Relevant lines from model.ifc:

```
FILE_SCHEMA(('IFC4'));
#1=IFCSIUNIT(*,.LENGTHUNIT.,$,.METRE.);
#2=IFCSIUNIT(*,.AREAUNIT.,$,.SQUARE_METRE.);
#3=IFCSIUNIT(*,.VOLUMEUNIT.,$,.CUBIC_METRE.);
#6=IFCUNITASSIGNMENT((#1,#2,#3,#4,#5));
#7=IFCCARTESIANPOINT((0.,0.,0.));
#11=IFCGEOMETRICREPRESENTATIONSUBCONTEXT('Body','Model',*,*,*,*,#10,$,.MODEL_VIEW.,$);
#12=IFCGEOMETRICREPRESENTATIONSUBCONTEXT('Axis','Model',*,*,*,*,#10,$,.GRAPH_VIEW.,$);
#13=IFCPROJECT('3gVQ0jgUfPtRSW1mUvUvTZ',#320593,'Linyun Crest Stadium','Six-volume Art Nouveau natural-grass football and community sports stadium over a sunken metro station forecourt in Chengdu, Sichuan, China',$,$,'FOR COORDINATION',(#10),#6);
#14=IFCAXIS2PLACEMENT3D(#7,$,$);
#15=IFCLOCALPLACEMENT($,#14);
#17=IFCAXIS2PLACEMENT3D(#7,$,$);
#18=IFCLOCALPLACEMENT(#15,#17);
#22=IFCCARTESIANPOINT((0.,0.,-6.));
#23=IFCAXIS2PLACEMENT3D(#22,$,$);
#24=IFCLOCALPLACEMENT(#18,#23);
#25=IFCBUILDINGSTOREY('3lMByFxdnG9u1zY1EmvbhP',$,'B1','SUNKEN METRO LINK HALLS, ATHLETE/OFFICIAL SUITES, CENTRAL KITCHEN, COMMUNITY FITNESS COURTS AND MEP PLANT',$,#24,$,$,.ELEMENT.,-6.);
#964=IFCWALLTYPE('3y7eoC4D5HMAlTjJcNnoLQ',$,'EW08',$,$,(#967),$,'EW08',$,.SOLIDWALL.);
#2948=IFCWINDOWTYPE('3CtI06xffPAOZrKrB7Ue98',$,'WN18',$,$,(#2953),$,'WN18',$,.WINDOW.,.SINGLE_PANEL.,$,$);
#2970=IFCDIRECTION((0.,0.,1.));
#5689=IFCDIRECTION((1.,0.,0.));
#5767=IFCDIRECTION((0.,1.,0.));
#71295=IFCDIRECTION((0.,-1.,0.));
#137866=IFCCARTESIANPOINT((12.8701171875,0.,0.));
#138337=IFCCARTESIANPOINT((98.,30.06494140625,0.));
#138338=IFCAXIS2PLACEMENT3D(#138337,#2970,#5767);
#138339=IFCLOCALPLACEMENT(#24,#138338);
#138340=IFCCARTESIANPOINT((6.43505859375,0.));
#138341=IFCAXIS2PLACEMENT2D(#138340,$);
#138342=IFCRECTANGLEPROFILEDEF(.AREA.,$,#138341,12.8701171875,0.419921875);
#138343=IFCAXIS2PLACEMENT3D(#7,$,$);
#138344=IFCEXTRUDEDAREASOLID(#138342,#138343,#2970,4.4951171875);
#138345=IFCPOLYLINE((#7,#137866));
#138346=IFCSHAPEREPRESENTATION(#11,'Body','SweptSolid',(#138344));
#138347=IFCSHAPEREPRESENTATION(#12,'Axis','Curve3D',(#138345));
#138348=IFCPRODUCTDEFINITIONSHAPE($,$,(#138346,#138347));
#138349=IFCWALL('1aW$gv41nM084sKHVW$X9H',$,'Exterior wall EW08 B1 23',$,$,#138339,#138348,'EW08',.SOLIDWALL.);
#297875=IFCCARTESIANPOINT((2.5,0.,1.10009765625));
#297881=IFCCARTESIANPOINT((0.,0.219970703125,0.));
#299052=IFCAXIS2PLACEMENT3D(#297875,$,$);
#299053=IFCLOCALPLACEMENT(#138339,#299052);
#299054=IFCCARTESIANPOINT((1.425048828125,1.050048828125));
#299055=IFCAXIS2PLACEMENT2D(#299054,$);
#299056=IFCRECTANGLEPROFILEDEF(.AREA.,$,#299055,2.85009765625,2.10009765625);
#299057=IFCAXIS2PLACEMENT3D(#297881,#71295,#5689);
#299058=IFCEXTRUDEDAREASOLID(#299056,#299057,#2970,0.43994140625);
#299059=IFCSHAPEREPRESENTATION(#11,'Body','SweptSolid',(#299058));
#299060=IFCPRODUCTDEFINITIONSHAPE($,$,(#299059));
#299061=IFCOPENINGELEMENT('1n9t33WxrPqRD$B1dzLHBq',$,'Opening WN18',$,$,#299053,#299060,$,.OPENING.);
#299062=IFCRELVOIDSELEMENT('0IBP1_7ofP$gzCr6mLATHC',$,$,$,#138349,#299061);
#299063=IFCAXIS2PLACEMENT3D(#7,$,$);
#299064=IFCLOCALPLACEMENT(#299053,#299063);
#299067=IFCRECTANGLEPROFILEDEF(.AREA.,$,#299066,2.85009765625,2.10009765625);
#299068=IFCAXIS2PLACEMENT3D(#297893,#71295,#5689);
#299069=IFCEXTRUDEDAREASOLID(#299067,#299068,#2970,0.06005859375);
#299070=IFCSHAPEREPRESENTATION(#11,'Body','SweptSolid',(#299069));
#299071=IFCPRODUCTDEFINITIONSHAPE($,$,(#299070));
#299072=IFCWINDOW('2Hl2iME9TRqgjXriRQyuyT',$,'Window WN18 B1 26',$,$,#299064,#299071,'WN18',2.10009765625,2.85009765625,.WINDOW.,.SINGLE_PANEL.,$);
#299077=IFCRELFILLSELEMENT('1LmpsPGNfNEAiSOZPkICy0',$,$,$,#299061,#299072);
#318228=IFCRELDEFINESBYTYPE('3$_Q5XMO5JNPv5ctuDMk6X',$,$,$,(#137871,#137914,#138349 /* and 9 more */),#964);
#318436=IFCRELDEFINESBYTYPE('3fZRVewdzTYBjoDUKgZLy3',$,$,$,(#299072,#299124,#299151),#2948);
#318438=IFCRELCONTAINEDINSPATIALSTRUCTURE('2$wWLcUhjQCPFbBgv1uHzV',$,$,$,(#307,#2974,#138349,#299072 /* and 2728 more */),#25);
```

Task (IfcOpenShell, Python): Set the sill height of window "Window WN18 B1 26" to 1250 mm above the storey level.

```python
import numpy as np
import ifcopenshell
import ifcopenshell.api.geometry
import ifcopenshell.geom
import ifcopenshell.util.element
import ifcopenshell.util.placement
import ifcopenshell.util.shape
import ifcopenshell.util.unit

model = ifcopenshell.open("model.ifc")
unit_scale = ifcopenshell.util.unit.calculate_unit_scale(model)

window = model.by_guid("2Hl2iME9TRqgjXriRQyuyT")
opening = window.FillsVoids[0].RelatingOpeningElement
storey = ifcopenshell.util.element.get_container(window, ifc_class="IfcBuildingStorey")
level = ifcopenshell.util.placement.get_local_placement(storey.ObjectPlacement)[2, 3]

# The opening's origin need not be at the sill, so measure its lowest point.
shape = ifcopenshell.geom.create_shape(ifcopenshell.geom.settings(), opening)
bottom = ifcopenshell.util.shape.get_shape_bottom_elevation(shape, shape.geometry) / unit_scale
dz = level + 1.25 - bottom

shift = np.array([0.0, 0.0, dz])
# The window is placed relative to its opening, so it follows when the opening moves.
matrix = ifcopenshell.util.placement.get_local_placement(opening.ObjectPlacement)
matrix[:3, 3] += shift
ifcopenshell.api.geometry.edit_object_placement(
    model, product=opening, matrix=matrix, is_si=False, should_transform_children=True
)

print(f"moved by {dz * unit_scale:+.3f} m")

model.write("model_v2.ifc")
```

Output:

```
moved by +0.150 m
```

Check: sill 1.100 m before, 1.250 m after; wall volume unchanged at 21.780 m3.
